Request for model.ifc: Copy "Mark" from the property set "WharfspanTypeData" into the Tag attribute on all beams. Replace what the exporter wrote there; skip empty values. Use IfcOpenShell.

First a look at what the model holds.

```python
import ifcopenshell
import ifcopenshell.util.element

model = ifcopenshell.open("model.ifc")
print(model.schema)
beams = model.by_type("IfcBeam")
print(len(beams), "beams")
for e in beams[:8]:
    source = ifcopenshell.util.element.get_pset(e, "WharfspanTypeData", "Mark")
    target = e.Tag
    print(e.id(), repr(source), repr(target), sep=" | ")
```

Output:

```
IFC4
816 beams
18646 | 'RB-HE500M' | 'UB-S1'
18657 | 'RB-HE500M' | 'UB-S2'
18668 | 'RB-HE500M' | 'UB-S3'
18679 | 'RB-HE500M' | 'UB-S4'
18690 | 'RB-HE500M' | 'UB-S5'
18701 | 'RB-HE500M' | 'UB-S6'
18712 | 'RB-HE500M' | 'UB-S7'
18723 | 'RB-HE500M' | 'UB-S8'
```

```python
import ifcopenshell
import ifcopenshell.util.element

model = ifcopenshell.open("model.ifc")

count = 0
for e in model.by_type("IfcBeam"):
    value = ifcopenshell.util.element.get_pset(e, "WharfspanTypeData", "Mark")
    current = e.Tag
    if not value or not value.strip() or current == value:
        continue
    e.Tag = value
    count += 1

print(count, "beams updated")

model.write("model-out.ifc")
```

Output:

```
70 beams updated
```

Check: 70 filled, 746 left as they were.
